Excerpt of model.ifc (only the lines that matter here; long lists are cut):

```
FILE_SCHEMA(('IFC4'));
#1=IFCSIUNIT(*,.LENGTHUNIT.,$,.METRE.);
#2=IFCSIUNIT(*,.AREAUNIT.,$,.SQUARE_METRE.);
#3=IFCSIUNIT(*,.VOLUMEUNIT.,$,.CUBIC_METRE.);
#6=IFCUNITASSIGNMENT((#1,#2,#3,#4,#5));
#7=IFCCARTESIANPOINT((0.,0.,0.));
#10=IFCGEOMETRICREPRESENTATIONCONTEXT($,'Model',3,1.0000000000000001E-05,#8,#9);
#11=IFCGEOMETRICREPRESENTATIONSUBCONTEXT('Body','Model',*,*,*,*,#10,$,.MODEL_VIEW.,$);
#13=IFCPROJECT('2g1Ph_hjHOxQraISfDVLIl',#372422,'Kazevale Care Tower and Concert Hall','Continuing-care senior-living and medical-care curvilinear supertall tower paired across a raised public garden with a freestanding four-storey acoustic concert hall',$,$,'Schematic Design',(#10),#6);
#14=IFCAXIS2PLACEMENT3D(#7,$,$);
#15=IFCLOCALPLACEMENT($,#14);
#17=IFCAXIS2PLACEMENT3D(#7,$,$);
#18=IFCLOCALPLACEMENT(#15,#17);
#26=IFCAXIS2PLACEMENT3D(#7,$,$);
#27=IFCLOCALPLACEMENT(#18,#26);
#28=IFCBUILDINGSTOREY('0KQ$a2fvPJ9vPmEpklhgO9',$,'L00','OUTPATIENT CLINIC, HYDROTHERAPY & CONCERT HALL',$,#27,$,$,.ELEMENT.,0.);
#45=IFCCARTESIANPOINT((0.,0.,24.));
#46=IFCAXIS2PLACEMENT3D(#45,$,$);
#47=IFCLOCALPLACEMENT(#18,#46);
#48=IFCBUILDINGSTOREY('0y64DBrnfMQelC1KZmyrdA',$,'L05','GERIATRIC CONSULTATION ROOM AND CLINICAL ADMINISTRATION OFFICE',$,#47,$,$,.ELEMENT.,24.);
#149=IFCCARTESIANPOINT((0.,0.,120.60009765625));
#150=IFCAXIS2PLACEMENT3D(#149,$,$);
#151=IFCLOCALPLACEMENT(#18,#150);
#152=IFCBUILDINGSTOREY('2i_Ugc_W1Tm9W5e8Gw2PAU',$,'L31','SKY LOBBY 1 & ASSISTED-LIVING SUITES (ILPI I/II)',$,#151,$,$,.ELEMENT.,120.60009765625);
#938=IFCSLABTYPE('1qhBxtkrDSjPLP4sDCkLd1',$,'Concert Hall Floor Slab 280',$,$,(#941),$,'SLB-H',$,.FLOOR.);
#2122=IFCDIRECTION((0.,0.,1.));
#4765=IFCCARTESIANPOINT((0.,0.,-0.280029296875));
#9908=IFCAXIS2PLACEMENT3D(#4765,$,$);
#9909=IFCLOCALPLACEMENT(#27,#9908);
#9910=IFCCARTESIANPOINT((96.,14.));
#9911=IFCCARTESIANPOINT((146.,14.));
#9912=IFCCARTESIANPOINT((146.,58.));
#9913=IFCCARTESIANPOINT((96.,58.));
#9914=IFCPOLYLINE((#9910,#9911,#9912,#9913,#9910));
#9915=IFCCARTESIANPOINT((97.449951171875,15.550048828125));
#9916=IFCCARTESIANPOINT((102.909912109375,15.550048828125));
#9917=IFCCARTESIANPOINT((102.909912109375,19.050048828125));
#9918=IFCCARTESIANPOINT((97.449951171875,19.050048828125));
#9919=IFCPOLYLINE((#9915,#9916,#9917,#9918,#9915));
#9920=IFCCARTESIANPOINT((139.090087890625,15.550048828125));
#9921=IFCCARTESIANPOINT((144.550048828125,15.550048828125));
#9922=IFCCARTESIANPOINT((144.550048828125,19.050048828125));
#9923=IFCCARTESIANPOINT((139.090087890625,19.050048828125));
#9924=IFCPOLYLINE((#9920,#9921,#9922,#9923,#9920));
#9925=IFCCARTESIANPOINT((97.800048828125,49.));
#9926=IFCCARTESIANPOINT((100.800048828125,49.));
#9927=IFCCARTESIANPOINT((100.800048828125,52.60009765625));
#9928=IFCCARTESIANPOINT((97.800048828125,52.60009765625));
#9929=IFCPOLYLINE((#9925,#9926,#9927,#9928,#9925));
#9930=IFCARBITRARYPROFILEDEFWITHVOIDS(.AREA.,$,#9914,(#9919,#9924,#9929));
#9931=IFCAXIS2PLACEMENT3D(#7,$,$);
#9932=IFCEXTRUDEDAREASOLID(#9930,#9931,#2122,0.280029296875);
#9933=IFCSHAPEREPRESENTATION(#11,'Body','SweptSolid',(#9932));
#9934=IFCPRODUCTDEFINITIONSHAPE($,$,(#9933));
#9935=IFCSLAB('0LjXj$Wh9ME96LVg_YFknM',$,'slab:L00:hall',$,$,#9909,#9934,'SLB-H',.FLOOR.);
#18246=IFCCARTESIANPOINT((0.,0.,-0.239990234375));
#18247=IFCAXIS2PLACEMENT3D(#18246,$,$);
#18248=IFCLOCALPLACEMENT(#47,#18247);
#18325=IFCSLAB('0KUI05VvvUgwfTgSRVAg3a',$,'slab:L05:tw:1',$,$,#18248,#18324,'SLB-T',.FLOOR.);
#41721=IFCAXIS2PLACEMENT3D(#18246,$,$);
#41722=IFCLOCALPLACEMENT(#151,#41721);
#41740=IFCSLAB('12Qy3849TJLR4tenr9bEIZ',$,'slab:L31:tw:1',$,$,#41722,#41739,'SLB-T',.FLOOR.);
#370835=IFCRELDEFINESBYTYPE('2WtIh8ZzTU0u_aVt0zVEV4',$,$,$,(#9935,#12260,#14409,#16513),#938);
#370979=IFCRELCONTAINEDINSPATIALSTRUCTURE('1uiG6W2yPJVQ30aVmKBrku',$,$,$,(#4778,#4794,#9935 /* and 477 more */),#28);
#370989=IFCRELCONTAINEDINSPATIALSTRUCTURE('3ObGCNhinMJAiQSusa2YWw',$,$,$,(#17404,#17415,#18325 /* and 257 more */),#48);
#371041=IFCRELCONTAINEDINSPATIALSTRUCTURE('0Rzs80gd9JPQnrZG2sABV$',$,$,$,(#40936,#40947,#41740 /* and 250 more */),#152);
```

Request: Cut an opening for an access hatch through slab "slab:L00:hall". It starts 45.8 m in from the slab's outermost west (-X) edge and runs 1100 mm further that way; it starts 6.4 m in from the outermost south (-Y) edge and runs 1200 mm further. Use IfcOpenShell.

```python
import numpy as np
import ifcopenshell
import ifcopenshell.api.feature
import ifcopenshell.api.geometry
import ifcopenshell.api.root
import ifcopenshell.geom
import ifcopenshell.util.placement
import ifcopenshell.util.representation
import ifcopenshell.util.shape
import ifcopenshell.util.unit

model = ifcopenshell.open("model.ifc")
unit_scale = ifcopenshell.util.unit.calculate_unit_scale(model)
settings = ifcopenshell.geom.settings()


def volume(element):
    """Net volume in cubic metres, openings subtracted."""
    shape = ifcopenshell.geom.create_shape(settings, element)
    return ifcopenshell.util.shape.get_volume(shape.geometry)


slab = model.by_guid("0LjXj$Wh9ME96LVg_YFknM")
before = volume(slab)

# Extent in the slab's own axes, in metres. The edges named are its -X and -Y sides.
slab_shape = ifcopenshell.geom.create_shape(settings, slab)
vertices = ifcopenshell.util.shape.get_vertices(slab_shape.geometry)
x_min, y_min, bottom = vertices.min(axis=0)
top = vertices[:, 2].max()

opening = ifcopenshell.api.root.create_entity(model, ifc_class="IfcOpeningElement", name="Access hatch opening", predefined_type="OPENING")
context = ifcopenshell.util.representation.get_context(model, "Model", "Body", "MODEL_VIEW")
width, depth = 1.1, 1.2
outline = [(0.0, 0.0), (width, 0.0), (width, depth), (0.0, depth), (0.0, 0.0)]
# Overshoot both faces by 50 mm so the cut is clean.
shape = ifcopenshell.api.geometry.add_slab_representation(
    model, context=context, depth=top - bottom + 0.1, polyline=outline
)
ifcopenshell.api.geometry.assign_representation(model, product=opening, representation=shape)

matrix = ifcopenshell.util.placement.get_local_placement(slab.ObjectPlacement)
matrix[:, 3] = matrix @ np.append(np.array([x_min + 45.8, y_min + 6.4, bottom - 0.05]) / unit_scale, 1.0)
ifcopenshell.api.geometry.edit_object_placement(model, product=opening, matrix=matrix, is_si=False)
ifcopenshell.api.feature.add_feature(model, feature=opening, element=slab)

after = volume(slab)

print(f"slab volume {before:.3f} -> {after:.3f} m3")

model.write("model_rev.ifc")
```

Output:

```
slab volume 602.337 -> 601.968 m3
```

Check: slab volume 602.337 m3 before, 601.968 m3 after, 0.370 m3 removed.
